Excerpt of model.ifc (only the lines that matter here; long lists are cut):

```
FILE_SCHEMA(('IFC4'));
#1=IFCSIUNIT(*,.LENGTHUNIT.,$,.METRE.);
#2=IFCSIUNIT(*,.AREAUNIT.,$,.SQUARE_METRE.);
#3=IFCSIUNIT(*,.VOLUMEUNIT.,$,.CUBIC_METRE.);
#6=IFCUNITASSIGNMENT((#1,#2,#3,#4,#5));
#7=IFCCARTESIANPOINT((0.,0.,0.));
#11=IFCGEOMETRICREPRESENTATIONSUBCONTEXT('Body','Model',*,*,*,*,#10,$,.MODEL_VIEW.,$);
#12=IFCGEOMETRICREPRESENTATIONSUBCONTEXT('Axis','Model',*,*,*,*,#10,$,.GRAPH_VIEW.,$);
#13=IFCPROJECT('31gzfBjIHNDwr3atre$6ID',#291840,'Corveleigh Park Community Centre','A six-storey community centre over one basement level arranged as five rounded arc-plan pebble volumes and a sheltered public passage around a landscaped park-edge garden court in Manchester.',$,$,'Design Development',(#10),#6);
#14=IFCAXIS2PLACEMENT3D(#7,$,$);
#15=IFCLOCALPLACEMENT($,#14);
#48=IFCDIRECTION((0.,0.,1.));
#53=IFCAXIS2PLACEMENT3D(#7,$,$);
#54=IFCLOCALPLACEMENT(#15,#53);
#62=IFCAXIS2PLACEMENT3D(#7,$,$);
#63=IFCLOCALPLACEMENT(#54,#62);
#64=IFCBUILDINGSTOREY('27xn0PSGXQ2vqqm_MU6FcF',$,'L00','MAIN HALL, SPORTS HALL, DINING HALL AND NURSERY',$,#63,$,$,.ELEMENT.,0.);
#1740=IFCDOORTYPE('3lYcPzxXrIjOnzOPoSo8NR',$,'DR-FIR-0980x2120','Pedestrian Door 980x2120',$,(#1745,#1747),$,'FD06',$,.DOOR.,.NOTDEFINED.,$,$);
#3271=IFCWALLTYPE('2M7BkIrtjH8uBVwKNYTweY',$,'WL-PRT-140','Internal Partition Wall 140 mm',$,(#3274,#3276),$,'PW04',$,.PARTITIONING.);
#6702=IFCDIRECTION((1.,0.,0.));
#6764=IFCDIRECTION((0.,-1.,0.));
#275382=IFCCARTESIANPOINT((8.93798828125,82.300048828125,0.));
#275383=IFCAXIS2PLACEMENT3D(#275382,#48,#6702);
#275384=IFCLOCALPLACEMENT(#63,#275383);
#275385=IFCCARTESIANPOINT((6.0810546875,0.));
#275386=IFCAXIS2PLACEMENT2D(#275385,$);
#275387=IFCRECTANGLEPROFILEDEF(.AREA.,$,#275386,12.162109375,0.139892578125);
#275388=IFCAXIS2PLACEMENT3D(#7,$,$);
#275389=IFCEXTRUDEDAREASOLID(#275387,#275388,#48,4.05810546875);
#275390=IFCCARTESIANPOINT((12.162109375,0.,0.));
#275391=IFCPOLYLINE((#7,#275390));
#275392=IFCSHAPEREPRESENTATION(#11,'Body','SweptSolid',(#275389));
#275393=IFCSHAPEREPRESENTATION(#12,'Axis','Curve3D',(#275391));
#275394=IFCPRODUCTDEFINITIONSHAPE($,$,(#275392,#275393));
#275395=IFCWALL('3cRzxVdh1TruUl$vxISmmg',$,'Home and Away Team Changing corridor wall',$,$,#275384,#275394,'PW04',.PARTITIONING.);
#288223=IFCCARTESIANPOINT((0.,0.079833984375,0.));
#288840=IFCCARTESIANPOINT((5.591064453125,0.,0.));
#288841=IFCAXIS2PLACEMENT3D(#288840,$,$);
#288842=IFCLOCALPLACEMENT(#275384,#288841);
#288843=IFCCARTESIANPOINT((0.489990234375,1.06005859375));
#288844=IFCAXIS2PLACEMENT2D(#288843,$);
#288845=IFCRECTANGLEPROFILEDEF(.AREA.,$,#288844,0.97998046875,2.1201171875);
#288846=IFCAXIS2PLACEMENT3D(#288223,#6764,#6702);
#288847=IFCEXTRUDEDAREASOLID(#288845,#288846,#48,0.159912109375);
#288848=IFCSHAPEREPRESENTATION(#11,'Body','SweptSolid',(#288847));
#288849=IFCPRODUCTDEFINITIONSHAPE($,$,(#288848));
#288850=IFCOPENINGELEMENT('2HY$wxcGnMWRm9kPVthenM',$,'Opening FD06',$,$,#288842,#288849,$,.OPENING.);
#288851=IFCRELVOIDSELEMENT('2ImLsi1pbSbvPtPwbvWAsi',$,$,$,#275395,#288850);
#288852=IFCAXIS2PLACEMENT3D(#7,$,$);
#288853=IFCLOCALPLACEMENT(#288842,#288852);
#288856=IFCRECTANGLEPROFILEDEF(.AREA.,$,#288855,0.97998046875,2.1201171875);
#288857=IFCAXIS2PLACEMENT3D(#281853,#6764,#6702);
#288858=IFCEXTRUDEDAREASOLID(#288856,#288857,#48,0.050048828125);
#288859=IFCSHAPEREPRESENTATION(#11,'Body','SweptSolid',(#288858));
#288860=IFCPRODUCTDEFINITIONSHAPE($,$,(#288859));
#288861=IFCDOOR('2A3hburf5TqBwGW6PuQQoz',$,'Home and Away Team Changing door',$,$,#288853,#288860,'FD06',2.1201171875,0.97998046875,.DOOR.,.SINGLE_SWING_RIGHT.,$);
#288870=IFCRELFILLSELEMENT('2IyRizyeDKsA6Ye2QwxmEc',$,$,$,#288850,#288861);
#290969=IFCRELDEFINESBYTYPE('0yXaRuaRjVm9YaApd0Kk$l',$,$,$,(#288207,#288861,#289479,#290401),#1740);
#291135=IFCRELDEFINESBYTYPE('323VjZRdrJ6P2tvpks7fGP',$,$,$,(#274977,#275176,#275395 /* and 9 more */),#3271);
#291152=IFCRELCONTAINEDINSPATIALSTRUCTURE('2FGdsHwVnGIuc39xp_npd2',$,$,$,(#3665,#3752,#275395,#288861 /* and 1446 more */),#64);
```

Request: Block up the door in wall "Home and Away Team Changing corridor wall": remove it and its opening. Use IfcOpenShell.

```python
import ifcopenshell
import ifcopenshell.api.feature
import ifcopenshell.api.root
import ifcopenshell.geom
import ifcopenshell.util.shape

model = ifcopenshell.open("model.ifc")
settings = ifcopenshell.geom.settings()


def volume(element):
    """Net volume in cubic metres, openings subtracted."""
    shape = ifcopenshell.geom.create_shape(settings, element)
    return ifcopenshell.util.shape.get_volume(shape.geometry)


door = model.by_guid("2A3hburf5TqBwGW6PuQQoz")
opening = door.FillsVoids[0].RelatingOpeningElement
wall = opening.VoidsElements[0].RelatingBuildingElement
before = volume(wall)

ifcopenshell.api.root.remove_product(model, product=door)
ifcopenshell.api.feature.remove_feature(model, feature=opening)

after = volume(wall)

print(f"wall volume {before:.3f} -> {after:.3f} m3")

model.write("model_v2.ifc")
```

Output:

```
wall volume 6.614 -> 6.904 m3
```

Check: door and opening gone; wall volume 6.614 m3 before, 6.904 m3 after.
